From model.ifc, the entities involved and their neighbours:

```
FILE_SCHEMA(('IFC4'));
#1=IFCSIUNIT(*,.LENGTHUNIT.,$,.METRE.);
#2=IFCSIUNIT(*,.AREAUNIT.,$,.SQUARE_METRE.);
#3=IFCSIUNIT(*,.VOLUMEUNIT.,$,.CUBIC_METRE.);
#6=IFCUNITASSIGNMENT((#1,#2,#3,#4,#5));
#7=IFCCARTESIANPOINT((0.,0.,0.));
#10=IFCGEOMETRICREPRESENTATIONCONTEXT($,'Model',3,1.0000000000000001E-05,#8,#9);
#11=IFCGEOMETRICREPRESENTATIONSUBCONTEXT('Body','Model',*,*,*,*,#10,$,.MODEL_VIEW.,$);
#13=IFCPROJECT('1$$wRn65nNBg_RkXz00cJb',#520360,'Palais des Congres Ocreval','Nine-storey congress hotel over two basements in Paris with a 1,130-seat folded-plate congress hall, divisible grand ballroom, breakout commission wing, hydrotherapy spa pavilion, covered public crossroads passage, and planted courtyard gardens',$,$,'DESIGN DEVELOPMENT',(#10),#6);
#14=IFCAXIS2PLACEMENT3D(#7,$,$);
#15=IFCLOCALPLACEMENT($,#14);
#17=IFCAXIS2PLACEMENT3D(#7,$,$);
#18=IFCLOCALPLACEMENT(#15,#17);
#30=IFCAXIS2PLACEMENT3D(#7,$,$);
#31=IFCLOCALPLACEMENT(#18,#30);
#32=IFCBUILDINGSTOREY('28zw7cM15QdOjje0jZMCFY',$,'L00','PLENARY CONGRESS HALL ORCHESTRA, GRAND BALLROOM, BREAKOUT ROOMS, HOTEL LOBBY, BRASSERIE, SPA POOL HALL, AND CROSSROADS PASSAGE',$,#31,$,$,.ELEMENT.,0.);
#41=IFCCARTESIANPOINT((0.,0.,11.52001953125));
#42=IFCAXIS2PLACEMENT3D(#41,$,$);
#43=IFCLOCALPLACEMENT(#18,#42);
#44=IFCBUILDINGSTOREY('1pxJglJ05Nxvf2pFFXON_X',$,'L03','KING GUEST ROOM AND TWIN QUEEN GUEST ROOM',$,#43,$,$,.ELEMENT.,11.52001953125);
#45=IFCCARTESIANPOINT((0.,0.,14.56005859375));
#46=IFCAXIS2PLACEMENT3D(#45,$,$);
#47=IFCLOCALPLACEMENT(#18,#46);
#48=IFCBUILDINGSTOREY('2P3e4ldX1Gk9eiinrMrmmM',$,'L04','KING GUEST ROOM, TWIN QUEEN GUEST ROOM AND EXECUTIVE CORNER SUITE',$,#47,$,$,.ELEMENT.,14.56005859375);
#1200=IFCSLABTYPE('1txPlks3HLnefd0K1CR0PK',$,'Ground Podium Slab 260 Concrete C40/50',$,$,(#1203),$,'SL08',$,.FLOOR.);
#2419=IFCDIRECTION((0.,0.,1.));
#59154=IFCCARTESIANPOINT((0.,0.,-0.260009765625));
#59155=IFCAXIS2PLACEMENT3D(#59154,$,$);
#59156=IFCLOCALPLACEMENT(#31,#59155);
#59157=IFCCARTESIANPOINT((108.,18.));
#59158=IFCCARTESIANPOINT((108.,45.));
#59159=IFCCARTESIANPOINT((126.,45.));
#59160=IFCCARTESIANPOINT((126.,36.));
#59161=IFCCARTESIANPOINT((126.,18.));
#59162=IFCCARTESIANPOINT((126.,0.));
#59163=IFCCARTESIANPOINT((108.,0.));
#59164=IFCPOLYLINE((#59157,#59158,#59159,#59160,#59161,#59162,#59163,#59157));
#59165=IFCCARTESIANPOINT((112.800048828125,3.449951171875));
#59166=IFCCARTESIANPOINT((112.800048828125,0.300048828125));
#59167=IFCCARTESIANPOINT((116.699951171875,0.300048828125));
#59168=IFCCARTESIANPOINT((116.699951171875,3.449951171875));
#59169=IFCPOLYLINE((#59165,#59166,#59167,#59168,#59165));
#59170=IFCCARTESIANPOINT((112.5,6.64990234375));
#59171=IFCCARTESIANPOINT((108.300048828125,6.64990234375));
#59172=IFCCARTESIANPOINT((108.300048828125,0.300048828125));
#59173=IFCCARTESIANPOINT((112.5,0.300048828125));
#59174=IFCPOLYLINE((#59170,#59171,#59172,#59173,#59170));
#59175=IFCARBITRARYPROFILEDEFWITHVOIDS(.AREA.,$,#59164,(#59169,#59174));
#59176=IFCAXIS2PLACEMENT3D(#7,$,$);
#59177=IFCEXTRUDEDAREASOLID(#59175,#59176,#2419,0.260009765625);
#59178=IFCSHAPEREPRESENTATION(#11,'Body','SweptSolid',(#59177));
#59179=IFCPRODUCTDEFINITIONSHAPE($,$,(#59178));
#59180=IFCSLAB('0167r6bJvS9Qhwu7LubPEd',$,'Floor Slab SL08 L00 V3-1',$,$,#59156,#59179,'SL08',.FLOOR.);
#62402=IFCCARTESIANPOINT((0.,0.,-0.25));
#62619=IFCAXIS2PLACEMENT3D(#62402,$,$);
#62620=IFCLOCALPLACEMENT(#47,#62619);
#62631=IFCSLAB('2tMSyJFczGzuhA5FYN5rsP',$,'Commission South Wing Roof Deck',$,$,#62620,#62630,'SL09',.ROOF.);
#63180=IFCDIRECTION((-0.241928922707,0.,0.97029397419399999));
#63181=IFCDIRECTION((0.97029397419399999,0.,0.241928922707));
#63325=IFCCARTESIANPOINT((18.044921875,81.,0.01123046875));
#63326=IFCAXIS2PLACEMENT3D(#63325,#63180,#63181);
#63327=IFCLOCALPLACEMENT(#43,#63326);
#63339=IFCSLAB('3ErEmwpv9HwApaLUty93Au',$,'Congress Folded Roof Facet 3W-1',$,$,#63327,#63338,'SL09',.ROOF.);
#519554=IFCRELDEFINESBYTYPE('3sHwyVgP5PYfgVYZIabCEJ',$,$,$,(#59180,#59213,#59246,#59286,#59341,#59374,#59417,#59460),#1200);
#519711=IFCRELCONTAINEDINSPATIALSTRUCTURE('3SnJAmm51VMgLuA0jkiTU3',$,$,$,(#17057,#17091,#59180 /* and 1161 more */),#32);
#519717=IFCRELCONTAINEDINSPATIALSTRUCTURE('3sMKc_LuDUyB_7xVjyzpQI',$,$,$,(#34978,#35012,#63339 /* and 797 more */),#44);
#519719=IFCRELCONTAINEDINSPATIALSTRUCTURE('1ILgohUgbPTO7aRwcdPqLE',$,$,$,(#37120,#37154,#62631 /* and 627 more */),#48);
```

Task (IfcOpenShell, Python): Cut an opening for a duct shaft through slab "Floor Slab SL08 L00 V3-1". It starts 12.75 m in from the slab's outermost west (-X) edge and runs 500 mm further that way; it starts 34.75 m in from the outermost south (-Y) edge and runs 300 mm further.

```python
import numpy as np
import ifcopenshell
import ifcopenshell.api.feature
import ifcopenshell.api.geometry
import ifcopenshell.api.root
import ifcopenshell.geom
import ifcopenshell.util.placement
import ifcopenshell.util.representation
import ifcopenshell.util.shape
import ifcopenshell.util.unit

model = ifcopenshell.open("model.ifc")
unit_scale = ifcopenshell.util.unit.calculate_unit_scale(model)
settings = ifcopenshell.geom.settings()


def volume(element):
    """Net volume in cubic metres, openings subtracted."""
    shape = ifcopenshell.geom.create_shape(settings, element)
    return ifcopenshell.util.shape.get_volume(shape.geometry)


slab = model.by_id(59180)
before = volume(slab)

# Extent in the slab's own axes, in metres. The edges named are its -X and -Y sides.
slab_shape = ifcopenshell.geom.create_shape(settings, slab)
vertices = ifcopenshell.util.shape.get_vertices(slab_shape.geometry)
x_min, y_min, bottom = vertices.min(axis=0)
top = vertices[:, 2].max()

opening = ifcopenshell.api.root.create_entity(model, ifc_class="IfcOpeningElement", name="Duct shaft opening", predefined_type="OPENING")
context = ifcopenshell.util.representation.get_context(model, "Model", "Body", "MODEL_VIEW")
width, depth = 0.5, 0.3
outline = [(0.0, 0.0), (width, 0.0), (width, depth), (0.0, depth), (0.0, 0.0)]
# Overshoot both faces by 50 mm so the cut is clean.
shape = ifcopenshell.api.geometry.add_slab_representation(
    model, context=context, depth=top - bottom + 0.1, polyline=outline
)
ifcopenshell.api.geometry.assign_representation(model, product=opening, representation=shape)

matrix = ifcopenshell.util.placement.get_local_placement(slab.ObjectPlacement)
matrix[:, 3] = matrix @ np.append(np.array([x_min + 12.75, y_min + 34.75, bottom - 0.05]) / unit_scale, 1.0)
ifcopenshell.api.geometry.edit_object_placement(model, product=opening, matrix=matrix, is_si=False)
ifcopenshell.api.feature.add_feature(model, feature=opening, element=slab)

after = volume(slab)

print(f"slab volume {before:.3f} -> {after:.3f} m3")

model.write("model-out.ifc")
```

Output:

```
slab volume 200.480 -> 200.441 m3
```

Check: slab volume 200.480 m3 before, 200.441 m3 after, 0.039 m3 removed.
